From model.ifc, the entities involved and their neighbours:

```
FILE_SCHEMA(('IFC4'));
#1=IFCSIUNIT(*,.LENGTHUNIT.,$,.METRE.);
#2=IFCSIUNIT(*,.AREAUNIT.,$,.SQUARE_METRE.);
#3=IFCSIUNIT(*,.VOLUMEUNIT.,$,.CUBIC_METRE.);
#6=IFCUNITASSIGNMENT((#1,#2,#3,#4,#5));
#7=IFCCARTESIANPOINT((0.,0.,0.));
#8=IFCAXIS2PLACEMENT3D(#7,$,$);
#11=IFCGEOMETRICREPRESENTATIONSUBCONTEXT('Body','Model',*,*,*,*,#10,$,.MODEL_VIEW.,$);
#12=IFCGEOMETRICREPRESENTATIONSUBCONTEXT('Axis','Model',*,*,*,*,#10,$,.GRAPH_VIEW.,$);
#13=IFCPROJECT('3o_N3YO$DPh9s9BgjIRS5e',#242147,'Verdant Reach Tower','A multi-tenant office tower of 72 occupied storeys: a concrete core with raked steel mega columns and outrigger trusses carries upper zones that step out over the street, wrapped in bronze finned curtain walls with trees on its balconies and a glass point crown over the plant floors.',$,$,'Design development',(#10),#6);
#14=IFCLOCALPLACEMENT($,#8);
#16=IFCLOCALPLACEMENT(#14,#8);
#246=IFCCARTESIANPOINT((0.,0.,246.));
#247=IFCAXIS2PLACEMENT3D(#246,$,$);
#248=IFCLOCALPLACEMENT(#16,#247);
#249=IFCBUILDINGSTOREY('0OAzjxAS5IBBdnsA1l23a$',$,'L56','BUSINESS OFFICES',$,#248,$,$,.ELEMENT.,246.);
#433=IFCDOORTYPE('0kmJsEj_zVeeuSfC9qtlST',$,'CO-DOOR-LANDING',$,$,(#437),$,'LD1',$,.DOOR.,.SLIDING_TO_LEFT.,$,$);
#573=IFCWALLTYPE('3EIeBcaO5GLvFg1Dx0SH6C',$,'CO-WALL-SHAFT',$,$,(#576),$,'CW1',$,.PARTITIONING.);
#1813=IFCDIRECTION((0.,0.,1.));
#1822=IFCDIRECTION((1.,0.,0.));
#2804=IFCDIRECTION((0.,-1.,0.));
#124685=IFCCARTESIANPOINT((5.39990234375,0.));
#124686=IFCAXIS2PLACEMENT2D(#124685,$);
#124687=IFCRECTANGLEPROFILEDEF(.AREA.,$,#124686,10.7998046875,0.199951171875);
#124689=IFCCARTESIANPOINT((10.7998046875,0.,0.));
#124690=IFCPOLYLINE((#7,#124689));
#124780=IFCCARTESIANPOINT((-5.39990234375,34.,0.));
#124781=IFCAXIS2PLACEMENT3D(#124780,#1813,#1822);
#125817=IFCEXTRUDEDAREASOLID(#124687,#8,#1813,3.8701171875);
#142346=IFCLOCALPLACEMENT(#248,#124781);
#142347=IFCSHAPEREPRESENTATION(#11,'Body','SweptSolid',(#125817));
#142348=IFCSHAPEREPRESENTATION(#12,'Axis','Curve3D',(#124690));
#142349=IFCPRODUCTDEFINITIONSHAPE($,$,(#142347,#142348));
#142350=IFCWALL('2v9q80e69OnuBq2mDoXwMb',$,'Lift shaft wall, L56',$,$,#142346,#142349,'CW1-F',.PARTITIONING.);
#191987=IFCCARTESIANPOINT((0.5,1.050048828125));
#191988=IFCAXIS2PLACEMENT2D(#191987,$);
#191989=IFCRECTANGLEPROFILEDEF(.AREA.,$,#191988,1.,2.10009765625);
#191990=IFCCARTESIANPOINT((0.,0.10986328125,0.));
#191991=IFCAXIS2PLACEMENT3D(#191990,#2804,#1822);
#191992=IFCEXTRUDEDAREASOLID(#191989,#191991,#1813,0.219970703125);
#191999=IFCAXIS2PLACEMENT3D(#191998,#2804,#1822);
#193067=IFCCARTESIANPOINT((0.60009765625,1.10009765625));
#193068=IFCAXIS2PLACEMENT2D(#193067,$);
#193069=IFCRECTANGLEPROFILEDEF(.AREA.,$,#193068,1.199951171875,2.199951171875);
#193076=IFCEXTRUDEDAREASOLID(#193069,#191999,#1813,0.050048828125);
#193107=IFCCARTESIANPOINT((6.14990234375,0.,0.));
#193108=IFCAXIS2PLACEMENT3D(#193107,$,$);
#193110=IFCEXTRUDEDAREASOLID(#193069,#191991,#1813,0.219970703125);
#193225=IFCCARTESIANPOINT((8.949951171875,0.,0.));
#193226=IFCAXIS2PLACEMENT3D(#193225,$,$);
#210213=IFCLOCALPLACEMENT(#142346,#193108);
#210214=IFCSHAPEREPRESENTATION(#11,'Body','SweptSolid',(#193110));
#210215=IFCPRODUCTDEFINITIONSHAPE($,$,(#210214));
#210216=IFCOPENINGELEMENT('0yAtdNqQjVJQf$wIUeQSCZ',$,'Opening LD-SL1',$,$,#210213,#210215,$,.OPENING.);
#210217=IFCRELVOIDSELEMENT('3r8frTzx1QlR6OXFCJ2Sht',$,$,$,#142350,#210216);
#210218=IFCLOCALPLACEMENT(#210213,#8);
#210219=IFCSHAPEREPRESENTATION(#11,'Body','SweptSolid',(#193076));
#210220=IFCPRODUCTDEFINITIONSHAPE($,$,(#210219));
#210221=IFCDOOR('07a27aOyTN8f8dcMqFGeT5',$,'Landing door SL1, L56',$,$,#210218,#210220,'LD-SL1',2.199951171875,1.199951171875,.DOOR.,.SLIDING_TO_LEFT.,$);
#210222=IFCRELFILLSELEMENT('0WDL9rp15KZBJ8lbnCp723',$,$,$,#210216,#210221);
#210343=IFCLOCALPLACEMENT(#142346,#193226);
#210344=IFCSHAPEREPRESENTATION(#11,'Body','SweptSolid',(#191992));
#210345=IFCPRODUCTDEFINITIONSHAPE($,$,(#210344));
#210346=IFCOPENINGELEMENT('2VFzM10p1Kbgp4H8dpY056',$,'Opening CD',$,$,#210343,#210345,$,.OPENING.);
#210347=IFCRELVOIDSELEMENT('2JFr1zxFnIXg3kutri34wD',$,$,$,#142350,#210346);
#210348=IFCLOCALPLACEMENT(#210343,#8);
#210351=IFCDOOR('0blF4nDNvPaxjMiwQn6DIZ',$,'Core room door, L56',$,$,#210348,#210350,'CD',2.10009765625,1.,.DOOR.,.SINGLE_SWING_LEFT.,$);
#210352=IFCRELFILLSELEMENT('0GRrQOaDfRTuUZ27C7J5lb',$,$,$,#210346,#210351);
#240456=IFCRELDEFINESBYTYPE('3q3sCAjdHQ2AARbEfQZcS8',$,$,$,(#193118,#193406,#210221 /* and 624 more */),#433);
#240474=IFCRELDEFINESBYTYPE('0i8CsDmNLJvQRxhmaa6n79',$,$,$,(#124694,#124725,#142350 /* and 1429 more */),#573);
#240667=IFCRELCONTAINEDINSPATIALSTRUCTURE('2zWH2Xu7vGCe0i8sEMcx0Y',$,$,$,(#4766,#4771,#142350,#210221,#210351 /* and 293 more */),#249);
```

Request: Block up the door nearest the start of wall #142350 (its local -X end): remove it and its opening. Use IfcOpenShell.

```python
import ifcopenshell
import ifcopenshell.api.feature
import ifcopenshell.api.root
import ifcopenshell.geom
import ifcopenshell.util.shape

model = ifcopenshell.open("model.ifc")
settings = ifcopenshell.geom.settings()


def volume(element):
    """Net volume in cubic metres, openings subtracted."""
    shape = ifcopenshell.geom.create_shape(settings, element)
    return ifcopenshell.util.shape.get_volume(shape.geometry)


door = model.by_id(210221)
opening = door.FillsVoids[0].RelatingOpeningElement
wall = opening.VoidsElements[0].RelatingBuildingElement
before = volume(wall)

ifcopenshell.api.root.remove_product(model, product=door)
ifcopenshell.api.feature.remove_feature(model, feature=opening)

after = volume(wall)

print(f"wall volume {before:.3f} -> {after:.3f} m3")

model.write("model_rev.ifc")
```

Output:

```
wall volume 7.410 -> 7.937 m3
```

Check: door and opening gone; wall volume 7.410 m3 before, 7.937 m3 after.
